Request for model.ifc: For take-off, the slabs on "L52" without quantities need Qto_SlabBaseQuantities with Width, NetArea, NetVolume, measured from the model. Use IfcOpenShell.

First a look at what the model holds.

```python
import ifcopenshell
import ifcopenshell.util.element
import ifcopenshell.util.unit

model = ifcopenshell.open("model.ifc")
print(model.schema)
for unit_type in ("LENGTHUNIT", "AREAUNIT", "VOLUMEUNIT"):
    print(unit_type, ifcopenshell.util.unit.calculate_unit_scale(model, unit_type))
storey = next(s for s in model.by_type("IfcBuildingStorey") if s.Name == "L52")
slabs = [e for e in ifcopenshell.util.element.get_decomposition(storey) if e.is_a("IfcSlab")]
for e in sorted(slabs, key=lambda e: e.id()):
    print(e.id(), e.is_a(), e.Name, list(ifcopenshell.util.element.get_psets(e, qtos_only=True)), sep=" | ")
```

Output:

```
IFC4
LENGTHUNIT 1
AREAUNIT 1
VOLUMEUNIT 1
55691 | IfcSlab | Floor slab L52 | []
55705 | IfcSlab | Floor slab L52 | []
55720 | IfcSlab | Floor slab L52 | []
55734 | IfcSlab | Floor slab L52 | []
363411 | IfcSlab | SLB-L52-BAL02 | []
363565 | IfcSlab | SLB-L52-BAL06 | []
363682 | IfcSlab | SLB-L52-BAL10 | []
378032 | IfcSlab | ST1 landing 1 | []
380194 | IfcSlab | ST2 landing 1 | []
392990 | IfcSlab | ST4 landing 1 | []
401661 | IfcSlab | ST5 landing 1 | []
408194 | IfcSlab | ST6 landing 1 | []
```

```python
import ifcopenshell
import ifcopenshell.api.pset
import ifcopenshell.geom
import ifcopenshell.util.element
import ifcopenshell.util.shape
import ifcopenshell.util.unit

model = ifcopenshell.open("model.ifc")
unit_scale = ifcopenshell.util.unit.calculate_unit_scale(model)
area_scale = ifcopenshell.util.unit.calculate_unit_scale(model, "AREAUNIT")
volume_scale = ifcopenshell.util.unit.calculate_unit_scale(model, "VOLUMEUNIT")
settings = ifcopenshell.geom.settings()

storey = next(s for s in model.by_type("IfcBuildingStorey") if s.Name == "L52")
slabs = [e for e in ifcopenshell.util.element.get_decomposition(storey) if e.is_a("IfcSlab")]

for e in sorted(slabs, key=lambda e: e.id()):
    if ifcopenshell.util.element.get_psets(e, qtos_only=True, should_inherit=False):
        continue
    # Geometry comes back in metres, in the element's own axes.
    shape = ifcopenshell.geom.create_shape(settings, e)
    values = {
        "Width": ifcopenshell.util.shape.get_z(shape.geometry) / unit_scale,
        "NetArea": ifcopenshell.util.shape.get_footprint_area(shape.geometry) / area_scale,
        "NetVolume": ifcopenshell.util.shape.get_volume(shape.geometry) / volume_scale,
    }
    qto = ifcopenshell.api.pset.add_qto(model, product=e, name="Qto_SlabBaseQuantities")
    ifcopenshell.api.pset.edit_qto(model, qto=qto, properties=values)
    print(e.id(), {k: round(v, 3) for k, v in values.items()})

model.write("model_updated.ifc")
```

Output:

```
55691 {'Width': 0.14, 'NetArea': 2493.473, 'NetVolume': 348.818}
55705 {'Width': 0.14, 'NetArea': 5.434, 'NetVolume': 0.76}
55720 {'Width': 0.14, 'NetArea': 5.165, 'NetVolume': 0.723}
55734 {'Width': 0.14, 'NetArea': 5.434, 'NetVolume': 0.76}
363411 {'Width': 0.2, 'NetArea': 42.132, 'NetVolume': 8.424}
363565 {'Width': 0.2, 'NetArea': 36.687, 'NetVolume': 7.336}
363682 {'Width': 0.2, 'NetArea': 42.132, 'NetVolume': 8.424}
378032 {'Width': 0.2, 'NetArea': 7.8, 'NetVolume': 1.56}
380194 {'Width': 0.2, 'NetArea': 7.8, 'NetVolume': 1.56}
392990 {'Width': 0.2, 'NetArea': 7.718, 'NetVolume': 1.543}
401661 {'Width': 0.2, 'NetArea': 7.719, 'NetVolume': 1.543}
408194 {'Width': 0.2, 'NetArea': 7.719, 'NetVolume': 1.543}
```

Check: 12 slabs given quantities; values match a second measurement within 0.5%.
